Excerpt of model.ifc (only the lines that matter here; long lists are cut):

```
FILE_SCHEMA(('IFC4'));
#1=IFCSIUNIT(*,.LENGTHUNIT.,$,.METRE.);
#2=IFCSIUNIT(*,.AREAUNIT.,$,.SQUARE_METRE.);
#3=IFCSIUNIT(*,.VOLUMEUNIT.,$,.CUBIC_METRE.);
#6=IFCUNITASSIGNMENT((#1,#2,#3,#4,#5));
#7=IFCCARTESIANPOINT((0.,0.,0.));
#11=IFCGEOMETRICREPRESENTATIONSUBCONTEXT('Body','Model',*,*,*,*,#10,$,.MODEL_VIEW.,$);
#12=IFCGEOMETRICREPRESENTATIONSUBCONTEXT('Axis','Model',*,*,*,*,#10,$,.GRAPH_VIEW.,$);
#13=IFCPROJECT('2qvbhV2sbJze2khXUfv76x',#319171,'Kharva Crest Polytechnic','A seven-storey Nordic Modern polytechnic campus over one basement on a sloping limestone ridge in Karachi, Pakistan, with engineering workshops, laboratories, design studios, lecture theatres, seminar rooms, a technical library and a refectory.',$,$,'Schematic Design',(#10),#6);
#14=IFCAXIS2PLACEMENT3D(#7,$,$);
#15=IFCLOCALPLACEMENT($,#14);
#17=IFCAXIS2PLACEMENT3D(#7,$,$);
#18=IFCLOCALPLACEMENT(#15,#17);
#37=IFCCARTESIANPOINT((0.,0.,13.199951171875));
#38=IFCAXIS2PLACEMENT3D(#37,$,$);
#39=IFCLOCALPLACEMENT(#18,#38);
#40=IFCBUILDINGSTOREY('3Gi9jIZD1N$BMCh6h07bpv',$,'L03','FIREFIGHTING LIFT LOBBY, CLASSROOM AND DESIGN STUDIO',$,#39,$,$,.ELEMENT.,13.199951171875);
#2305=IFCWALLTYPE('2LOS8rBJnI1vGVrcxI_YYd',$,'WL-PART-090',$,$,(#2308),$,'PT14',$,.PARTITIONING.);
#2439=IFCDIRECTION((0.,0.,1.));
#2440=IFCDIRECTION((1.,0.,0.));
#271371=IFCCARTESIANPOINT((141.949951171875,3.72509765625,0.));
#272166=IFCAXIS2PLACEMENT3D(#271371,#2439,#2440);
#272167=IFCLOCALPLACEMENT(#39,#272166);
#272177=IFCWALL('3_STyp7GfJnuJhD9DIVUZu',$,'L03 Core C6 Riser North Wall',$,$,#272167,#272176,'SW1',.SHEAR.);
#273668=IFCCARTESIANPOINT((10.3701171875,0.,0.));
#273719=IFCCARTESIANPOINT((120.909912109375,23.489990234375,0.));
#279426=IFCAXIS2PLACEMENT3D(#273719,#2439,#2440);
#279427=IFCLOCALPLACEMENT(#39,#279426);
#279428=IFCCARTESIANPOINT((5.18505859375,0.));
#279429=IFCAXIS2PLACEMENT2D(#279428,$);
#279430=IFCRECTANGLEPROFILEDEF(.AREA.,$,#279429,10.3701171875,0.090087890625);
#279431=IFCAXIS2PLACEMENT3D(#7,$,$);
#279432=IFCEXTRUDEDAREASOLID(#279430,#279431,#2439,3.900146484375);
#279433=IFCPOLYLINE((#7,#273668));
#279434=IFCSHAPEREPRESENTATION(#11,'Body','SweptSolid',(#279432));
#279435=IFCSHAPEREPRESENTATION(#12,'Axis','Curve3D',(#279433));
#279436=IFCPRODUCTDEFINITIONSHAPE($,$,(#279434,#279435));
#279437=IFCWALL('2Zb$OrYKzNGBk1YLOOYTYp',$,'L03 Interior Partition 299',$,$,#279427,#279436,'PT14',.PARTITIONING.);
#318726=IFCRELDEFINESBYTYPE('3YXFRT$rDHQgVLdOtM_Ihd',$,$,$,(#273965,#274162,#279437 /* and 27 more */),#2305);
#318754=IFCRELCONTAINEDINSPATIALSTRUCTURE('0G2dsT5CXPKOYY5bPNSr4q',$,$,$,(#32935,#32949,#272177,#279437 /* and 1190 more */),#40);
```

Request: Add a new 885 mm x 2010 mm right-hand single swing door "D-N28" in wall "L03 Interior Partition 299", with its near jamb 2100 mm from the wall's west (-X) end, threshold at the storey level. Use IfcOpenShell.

```python
import numpy as np
import ifcopenshell
import ifcopenshell.api.feature
import ifcopenshell.api.geometry
import ifcopenshell.api.root
import ifcopenshell.api.spatial
import ifcopenshell.geom
import ifcopenshell.util.element
import ifcopenshell.util.placement
import ifcopenshell.util.representation
import ifcopenshell.util.shape
import ifcopenshell.util.unit

model = ifcopenshell.open("model.ifc")
unit_scale = ifcopenshell.util.unit.calculate_unit_scale(model)
settings = ifcopenshell.geom.settings()


def volume(element):
    """Net volume in cubic metres, openings subtracted."""
    shape = ifcopenshell.geom.create_shape(settings, element)
    return ifcopenshell.util.shape.get_volume(shape.geometry)


wall = model.by_id(279437)
storey = ifcopenshell.util.element.get_container(wall, ifc_class="IfcBuildingStorey")
context = ifcopenshell.util.representation.get_context(model, "Model", "Body", "MODEL_VIEW")
before = volume(wall)

width, height, from_end, sill = 0.885, 2.01, 2.1, 0.0  # metres

# The wall runs along its own X axis, and the end named is its -X end.
wall_shape = ifcopenshell.geom.create_shape(settings, wall)
x, y, z = ifcopenshell.util.shape.get_vertices(wall_shape.geometry).T
start = x.min() + from_end
face, thickness = float(y.min()), float(y.max() - y.min())
wall_matrix = ifcopenshell.util.placement.get_local_placement(wall.ObjectPlacement)
level = ifcopenshell.util.placement.get_local_placement(storey.ObjectPlacement)[2, 3]


def in_wall(x, y):
    """Placement at x, y metres in the wall's axes, at sill height."""
    matrix = wall_matrix.copy()
    matrix[:, 3] = wall_matrix @ np.array([x / unit_scale, y / unit_scale, 0.0, 1.0])
    matrix[2, 3] = level + sill / unit_scale
    return matrix


# Opening: a box that overshoots both wall faces by 50 mm.
opening = ifcopenshell.api.root.create_entity(model, ifc_class="IfcOpeningElement", predefined_type="OPENING")
box = ifcopenshell.api.geometry.add_wall_representation(
    model, context=context, length=width, height=height, thickness=thickness + 0.1
)
ifcopenshell.api.geometry.assign_representation(model, product=opening, representation=box)
ifcopenshell.api.geometry.edit_object_placement(model, product=opening, matrix=in_wall(start, face - 0.05), is_si=False)
ifcopenshell.api.feature.add_feature(model, feature=opening, element=wall)

door = ifcopenshell.api.root.create_entity(model, ifc_class="IfcDoor", name="D-N28", predefined_type="DOOR")
door.OverallWidth, door.OverallHeight = width / unit_scale, height / unit_scale
door.OperationType = "SINGLE_SWING_RIGHT"
body = ifcopenshell.api.geometry.add_door_representation(
    model,
    context=context,
    overall_width=door.OverallWidth,
    overall_height=door.OverallHeight,
    operation_type="SINGLE_SWING_RIGHT",
    lining_properties={"LiningDepth": thickness / unit_scale, "ThresholdDepth": thickness / unit_scale},
)
ifcopenshell.api.geometry.assign_representation(model, product=door, representation=body)
ifcopenshell.api.spatial.assign_container(model, products=[door], relating_structure=storey)
ifcopenshell.api.feature.add_filling(model, opening=opening, element=door)

# The lining spans the wall, so the door starts at the wall face.
ifcopenshell.api.geometry.edit_object_placement(model, product=door, matrix=in_wall(start, face), is_si=False)

after = volume(wall)

print(f"wall volume {before:.3f} -> {after:.3f} m3")

model.write("model_rev.ifc")
```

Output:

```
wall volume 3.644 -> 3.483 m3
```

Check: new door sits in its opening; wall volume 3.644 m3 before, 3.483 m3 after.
